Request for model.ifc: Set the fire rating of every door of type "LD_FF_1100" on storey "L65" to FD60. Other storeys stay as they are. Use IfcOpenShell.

First a look at what the model holds.

```python
import ifcopenshell
import ifcopenshell.util.element

model = ifcopenshell.open("model.ifc")
print(model.schema)
storey = next(s for s in model.by_type("IfcBuildingStorey") if s.Name == "L65")
doors = [e for e in ifcopenshell.util.element.get_decomposition(storey) if e.is_a("IfcDoor")]
seen = {}
for e in doors:
    element_type = ifcopenshell.util.element.get_type(e)
    key = (element_type.Name if element_type != e and element_type else None, ifcopenshell.util.element.get_pset(e, "Pset_DoorCommon", "FireRating"))
    seen[key] = seen.get(key, 0) + 1
for (name, value), count in sorted(seen.items(), key=str):
    print(count, "x", name, "|", value)
```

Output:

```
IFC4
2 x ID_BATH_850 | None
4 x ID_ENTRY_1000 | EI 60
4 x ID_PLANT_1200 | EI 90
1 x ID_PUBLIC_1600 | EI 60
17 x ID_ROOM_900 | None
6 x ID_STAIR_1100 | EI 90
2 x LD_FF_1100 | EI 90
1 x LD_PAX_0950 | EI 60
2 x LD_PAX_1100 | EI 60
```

```python
import ifcopenshell
import ifcopenshell.api.pset
import ifcopenshell.util.element

model = ifcopenshell.open("model.ifc")

storey = next(s for s in model.by_type("IfcBuildingStorey") if s.Name == "L65")
doors = [e for e in ifcopenshell.util.element.get_decomposition(storey) if e.is_a("IfcDoor")]

count = 0
for e in doors:
    element_type = ifcopenshell.util.element.get_type(e)
    if element_type in (None, e) or element_type.Name != "LD_FF_1100":
        continue
    # add_pset returns the element's existing set when there is one.
    pset = ifcopenshell.api.pset.add_pset(model, product=e, name="Pset_DoorCommon")
    ifcopenshell.api.pset.edit_pset(model, pset=pset, properties={"FireRating": "FD60"})
    count += 1

print(count, "doors updated")

model.write("model-out.ifc")
```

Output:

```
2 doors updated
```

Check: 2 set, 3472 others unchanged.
